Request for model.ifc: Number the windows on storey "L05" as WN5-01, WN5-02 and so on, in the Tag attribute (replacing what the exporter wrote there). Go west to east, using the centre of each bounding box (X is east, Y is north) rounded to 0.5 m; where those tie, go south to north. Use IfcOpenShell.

First a look at what the model holds.

```python
import ifcopenshell
import ifcopenshell.util.element
import ifcopenshell.util.placement

model = ifcopenshell.open("model.ifc")
print(model.schema)
storey = next(s for s in model.by_type("IfcBuildingStorey") if s.Name == "L05")
windows = [e for e in ifcopenshell.util.element.get_decomposition(storey) if e.is_a("IfcWindow")]
for e in sorted(windows, key=lambda e: e.id()):
    origin = ifcopenshell.util.placement.get_local_placement(e.ObjectPlacement)[:3, 3]
    print(e.id(), e.Tag, e.Name, origin.round(2) + 0.0, sep=" | ")
```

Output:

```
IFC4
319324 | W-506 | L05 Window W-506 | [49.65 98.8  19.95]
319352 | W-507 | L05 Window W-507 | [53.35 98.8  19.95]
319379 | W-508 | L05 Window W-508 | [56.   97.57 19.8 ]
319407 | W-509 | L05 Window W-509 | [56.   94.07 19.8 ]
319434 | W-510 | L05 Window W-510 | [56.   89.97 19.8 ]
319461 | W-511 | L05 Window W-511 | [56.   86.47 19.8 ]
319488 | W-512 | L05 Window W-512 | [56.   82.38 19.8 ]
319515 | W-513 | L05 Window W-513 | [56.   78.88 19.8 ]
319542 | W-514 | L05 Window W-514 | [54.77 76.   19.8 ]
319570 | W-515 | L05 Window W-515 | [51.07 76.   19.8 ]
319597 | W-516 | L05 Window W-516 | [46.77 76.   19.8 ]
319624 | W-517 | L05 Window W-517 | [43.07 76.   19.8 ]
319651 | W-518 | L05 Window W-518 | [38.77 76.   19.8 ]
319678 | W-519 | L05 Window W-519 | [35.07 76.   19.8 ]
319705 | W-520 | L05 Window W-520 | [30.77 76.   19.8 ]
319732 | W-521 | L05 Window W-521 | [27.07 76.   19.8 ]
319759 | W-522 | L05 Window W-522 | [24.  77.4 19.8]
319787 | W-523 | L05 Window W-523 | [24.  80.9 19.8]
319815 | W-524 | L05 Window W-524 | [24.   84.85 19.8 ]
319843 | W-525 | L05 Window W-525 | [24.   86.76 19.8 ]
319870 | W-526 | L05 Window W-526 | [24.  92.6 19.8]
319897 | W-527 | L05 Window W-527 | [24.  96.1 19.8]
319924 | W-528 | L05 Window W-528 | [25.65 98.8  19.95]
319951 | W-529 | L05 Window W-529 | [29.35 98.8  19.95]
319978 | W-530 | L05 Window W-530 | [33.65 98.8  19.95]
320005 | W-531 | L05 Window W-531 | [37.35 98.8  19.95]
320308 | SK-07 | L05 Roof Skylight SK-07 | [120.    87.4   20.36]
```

```python
import ifcopenshell
import ifcopenshell.geom
import ifcopenshell.util.element
import ifcopenshell.util.shape

model = ifcopenshell.open("model.ifc")
settings = ifcopenshell.geom.settings()
settings.set("use-world-coords", True)


def centre(element):
    shape = ifcopenshell.geom.create_shape(settings, element)
    return ifcopenshell.util.shape.get_bbox_centroid(shape.geometry)


storey = next(s for s in model.by_type("IfcBuildingStorey") if s.Name == "L05")
windows = [e for e in ifcopenshell.util.element.get_decomposition(storey) if e.is_a("IfcWindow")]

# Insertion points can sit at a corner or the storey origin, so sort by the geometry (in metres).
centres = {e: centre(e) for e in windows}
windows.sort(key=lambda e: (round(centres[e][0] / 0.5), centres[e][1]))

for i, e in enumerate(windows, start=1):
    number = f"WN5-{i:02d}"
    e.Tag = number
    print(e.id(), number)

model.write("model_rev.ifc")
```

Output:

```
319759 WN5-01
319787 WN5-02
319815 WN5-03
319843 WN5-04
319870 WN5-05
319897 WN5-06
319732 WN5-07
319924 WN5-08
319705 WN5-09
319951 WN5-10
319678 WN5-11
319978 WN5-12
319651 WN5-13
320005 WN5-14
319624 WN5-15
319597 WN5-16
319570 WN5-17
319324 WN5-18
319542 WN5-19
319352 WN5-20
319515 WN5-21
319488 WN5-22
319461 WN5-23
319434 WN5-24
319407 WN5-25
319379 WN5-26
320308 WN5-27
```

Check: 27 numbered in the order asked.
